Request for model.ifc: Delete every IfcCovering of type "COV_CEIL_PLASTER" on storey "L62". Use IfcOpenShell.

First a look at what the model holds.

```python
import ifcopenshell
import ifcopenshell.util.element

model = ifcopenshell.open("model.ifc")
print(model.schema)
storey = next(s for s in model.by_type("IfcBuildingStorey") if s.Name == "L62")
coverings = [e for e in ifcopenshell.util.element.get_decomposition(storey) if e.is_a("IfcCovering")]
seen = {}
for e in coverings:
    element_type = ifcopenshell.util.element.get_type(e)
    name = element_type.Name if element_type not in (None, e) else None
    seen[name] = seen.get(name, 0) + 1
for name, count in sorted(seen.items(), key=str):
    print(count, "x", name)
```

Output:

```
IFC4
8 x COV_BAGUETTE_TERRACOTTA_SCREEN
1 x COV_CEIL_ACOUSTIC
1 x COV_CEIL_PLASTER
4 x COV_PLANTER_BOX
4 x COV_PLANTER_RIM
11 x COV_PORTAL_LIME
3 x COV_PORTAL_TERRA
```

```python
import ifcopenshell
import ifcopenshell.api.root
import ifcopenshell.util.element

model = ifcopenshell.open("model.ifc")

storey = next(s for s in model.by_type("IfcBuildingStorey") if s.Name == "L62")
coverings = [e for e in ifcopenshell.util.element.get_decomposition(storey) if e.is_a("IfcCovering")]
targets = [e for e in coverings if (t := ifcopenshell.util.element.get_type(e)) not in (None, e) and t.Name == "COV_CEIL_PLASTER"]

for e in targets:
    ifcopenshell.api.root.remove_product(model, product=e)
print(len(targets), "removed")

model.write("model_v2.ifc")
```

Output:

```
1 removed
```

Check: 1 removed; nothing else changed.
